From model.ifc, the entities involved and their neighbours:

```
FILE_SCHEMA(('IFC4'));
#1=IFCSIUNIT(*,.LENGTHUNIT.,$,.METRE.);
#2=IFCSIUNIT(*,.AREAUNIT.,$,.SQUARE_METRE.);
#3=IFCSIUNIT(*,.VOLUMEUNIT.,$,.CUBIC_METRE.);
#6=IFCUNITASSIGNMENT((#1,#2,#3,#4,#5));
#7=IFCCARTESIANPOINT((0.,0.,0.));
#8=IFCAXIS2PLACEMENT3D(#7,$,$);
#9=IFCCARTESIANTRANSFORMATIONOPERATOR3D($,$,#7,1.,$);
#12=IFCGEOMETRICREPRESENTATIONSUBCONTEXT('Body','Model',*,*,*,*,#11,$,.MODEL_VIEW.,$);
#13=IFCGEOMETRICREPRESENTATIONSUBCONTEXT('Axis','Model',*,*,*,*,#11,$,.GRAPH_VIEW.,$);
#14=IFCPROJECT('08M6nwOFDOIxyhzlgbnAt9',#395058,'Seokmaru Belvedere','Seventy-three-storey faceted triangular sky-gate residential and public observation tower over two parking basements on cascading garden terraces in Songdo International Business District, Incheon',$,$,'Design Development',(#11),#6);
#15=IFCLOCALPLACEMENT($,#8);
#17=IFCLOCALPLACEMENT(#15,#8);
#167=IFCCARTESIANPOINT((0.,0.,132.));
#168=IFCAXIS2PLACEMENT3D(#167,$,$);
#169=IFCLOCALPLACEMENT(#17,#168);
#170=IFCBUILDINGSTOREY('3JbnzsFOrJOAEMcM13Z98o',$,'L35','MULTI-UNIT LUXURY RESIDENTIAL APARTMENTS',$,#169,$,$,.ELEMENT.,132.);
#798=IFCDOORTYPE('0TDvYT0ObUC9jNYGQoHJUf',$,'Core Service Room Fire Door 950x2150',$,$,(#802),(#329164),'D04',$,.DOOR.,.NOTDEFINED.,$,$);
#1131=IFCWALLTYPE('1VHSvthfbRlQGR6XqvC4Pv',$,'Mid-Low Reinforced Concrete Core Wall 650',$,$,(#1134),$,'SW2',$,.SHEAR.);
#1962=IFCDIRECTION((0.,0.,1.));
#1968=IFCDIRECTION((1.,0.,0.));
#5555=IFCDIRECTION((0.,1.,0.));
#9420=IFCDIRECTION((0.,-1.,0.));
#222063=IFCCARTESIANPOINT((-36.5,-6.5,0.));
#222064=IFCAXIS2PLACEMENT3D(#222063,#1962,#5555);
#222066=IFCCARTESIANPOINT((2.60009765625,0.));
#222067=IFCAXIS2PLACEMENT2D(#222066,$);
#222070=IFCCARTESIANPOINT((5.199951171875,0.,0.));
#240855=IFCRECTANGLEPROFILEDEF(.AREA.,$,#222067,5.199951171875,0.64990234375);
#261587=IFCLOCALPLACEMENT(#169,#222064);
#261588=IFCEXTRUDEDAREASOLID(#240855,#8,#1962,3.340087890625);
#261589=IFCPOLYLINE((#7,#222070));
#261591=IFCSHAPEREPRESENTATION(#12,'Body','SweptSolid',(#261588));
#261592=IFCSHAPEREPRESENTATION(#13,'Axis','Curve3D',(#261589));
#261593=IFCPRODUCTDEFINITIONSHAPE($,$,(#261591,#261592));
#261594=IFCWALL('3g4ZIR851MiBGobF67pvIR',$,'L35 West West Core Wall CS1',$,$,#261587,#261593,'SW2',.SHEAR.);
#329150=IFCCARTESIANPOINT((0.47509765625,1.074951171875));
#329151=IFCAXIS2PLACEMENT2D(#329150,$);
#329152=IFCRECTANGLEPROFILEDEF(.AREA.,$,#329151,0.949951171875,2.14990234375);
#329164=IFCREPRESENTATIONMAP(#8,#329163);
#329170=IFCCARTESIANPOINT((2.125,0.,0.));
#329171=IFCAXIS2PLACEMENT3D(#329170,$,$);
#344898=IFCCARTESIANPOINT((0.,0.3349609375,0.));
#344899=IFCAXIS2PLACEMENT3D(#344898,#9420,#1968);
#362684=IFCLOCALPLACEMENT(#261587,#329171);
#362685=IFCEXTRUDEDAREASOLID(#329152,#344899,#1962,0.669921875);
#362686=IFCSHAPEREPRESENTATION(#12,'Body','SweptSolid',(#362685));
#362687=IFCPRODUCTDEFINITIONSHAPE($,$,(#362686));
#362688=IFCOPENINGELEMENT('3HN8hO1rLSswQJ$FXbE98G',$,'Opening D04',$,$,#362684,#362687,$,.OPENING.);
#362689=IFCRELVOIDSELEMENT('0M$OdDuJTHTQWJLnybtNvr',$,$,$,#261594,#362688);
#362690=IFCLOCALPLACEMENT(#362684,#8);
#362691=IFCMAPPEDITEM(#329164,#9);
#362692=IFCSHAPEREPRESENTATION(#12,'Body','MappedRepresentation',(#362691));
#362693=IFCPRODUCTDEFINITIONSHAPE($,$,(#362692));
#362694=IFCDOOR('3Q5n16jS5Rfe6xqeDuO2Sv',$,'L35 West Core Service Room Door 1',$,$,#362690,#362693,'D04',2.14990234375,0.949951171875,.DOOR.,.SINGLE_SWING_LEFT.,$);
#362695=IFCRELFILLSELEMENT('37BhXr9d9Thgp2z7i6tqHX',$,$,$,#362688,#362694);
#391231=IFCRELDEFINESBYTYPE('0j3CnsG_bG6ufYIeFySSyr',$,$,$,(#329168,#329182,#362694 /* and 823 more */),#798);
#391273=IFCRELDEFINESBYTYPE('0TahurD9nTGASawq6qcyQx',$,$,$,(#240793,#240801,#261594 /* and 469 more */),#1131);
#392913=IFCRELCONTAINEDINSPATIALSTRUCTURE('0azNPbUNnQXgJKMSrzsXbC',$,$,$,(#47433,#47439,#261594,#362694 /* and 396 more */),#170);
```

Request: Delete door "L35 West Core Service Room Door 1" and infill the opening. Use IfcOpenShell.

```python
import ifcopenshell
import ifcopenshell.api.feature
import ifcopenshell.api.root
import ifcopenshell.geom
import ifcopenshell.util.shape

model = ifcopenshell.open("model.ifc")
settings = ifcopenshell.geom.settings()


def volume(element):
    """Net volume in cubic metres, openings subtracted."""
    shape = ifcopenshell.geom.create_shape(settings, element)
    return ifcopenshell.util.shape.get_volume(shape.geometry)


door = model.by_guid("3Q5n16jS5Rfe6xqeDuO2Sv")
opening = door.FillsVoids[0].RelatingOpeningElement
wall = opening.VoidsElements[0].RelatingBuildingElement
before = volume(wall)

ifcopenshell.api.root.remove_product(model, product=door)
ifcopenshell.api.feature.remove_feature(model, feature=opening)

after = volume(wall)

print(f"wall volume {before:.3f} -> {after:.3f} m3")

model.write("model_rev.ifc")
```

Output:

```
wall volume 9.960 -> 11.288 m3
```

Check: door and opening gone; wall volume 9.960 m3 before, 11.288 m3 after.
